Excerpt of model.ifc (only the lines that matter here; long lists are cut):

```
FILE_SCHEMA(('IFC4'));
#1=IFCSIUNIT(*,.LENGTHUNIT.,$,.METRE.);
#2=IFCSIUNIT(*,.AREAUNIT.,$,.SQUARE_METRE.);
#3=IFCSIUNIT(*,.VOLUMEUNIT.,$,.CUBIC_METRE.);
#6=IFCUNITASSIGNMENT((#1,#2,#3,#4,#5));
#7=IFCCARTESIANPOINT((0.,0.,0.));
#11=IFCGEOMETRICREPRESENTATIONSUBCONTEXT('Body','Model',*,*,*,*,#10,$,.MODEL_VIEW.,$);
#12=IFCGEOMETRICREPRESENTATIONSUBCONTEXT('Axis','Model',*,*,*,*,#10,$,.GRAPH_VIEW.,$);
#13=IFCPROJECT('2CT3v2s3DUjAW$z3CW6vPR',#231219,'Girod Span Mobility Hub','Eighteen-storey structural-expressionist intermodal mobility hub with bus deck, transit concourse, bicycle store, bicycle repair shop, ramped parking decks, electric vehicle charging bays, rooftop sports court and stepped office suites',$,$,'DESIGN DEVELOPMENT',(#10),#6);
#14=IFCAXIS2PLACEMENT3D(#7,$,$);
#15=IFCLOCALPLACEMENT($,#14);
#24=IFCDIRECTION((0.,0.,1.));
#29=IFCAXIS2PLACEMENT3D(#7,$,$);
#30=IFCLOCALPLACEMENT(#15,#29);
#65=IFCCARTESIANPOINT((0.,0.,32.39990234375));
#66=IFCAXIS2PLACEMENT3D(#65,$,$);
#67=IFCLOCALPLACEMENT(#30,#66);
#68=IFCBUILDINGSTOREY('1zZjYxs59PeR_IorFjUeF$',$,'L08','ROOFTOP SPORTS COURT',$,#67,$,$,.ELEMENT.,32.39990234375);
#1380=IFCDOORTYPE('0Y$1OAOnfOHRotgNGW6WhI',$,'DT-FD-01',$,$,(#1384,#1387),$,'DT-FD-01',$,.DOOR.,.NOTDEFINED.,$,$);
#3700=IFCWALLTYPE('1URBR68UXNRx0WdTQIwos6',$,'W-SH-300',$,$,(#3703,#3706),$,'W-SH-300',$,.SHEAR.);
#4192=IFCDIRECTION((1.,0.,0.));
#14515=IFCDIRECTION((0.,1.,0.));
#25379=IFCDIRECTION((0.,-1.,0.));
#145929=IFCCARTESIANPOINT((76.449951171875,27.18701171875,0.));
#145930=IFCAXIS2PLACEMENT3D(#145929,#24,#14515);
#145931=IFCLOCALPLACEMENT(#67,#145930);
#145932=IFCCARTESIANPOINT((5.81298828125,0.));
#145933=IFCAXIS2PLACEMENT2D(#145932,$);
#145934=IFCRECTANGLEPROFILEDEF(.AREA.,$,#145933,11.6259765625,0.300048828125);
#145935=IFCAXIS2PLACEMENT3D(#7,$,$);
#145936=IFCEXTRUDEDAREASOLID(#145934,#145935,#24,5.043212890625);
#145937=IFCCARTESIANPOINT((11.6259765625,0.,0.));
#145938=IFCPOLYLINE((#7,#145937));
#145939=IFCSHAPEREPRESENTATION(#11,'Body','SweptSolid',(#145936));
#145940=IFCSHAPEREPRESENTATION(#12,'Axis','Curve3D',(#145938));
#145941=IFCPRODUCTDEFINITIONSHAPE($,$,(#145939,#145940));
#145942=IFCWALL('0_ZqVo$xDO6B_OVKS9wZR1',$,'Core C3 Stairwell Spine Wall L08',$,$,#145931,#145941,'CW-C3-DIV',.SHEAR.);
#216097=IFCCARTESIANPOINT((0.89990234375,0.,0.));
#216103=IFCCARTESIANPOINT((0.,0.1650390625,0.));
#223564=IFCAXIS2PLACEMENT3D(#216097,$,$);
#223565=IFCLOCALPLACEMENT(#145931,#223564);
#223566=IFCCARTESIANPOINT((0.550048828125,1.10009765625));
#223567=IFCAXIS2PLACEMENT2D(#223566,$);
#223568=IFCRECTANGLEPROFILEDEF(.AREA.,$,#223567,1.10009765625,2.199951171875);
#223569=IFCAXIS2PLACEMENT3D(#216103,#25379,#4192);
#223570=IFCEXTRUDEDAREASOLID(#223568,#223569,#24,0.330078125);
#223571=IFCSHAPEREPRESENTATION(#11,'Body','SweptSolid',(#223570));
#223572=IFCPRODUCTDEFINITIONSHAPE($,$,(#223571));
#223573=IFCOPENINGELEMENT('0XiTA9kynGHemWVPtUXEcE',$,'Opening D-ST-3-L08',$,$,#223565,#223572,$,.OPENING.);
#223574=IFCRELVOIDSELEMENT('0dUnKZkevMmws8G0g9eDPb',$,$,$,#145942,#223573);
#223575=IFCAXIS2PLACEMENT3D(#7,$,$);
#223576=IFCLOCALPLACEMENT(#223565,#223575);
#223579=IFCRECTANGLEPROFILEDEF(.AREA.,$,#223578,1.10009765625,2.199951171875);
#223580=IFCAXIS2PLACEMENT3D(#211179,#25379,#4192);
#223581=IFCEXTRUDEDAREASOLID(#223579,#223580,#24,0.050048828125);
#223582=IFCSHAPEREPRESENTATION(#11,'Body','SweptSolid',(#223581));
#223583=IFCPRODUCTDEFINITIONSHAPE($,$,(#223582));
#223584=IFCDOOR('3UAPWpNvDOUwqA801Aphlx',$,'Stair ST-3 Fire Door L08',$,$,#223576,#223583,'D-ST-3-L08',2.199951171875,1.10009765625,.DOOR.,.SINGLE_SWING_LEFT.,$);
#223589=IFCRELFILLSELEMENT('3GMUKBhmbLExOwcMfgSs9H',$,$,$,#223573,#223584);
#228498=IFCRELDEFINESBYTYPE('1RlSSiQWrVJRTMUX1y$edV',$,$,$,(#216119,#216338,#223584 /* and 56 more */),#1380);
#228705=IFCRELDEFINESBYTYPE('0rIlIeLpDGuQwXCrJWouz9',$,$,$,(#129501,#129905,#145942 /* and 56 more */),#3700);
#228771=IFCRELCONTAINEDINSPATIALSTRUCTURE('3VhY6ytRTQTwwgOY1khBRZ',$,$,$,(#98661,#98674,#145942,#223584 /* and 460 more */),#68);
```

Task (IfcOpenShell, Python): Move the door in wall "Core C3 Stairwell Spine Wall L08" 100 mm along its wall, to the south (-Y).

```python
import ifcopenshell
import ifcopenshell.api.geometry
import ifcopenshell.util.placement

model = ifcopenshell.open("model.ifc")

door = model.by_guid("3UAPWpNvDOUwqA801Aphlx")
opening = door.FillsVoids[0].RelatingOpeningElement
wall = opening.VoidsElements[0].RelatingBuildingElement

wall_matrix = ifcopenshell.util.placement.get_local_placement(wall.ObjectPlacement)
shift = wall_matrix[:3, 0] * -0.1
before = ifcopenshell.util.placement.get_local_placement(door.ObjectPlacement)[:3, 3].copy()

# The door is placed relative to its opening, so it follows when the opening moves.
matrix = ifcopenshell.util.placement.get_local_placement(opening.ObjectPlacement)
matrix[:3, 3] += shift
ifcopenshell.api.geometry.edit_object_placement(
    model, product=opening, matrix=matrix, is_si=False, should_transform_children=True
)

after = ifcopenshell.util.placement.get_local_placement(door.ObjectPlacement)[:3, 3]
print("door moved by", (after - before).round(3) + 0.0)

model.write("model_v2.ifc")
```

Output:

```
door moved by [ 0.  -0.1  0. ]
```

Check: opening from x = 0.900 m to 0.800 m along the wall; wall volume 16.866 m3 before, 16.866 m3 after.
